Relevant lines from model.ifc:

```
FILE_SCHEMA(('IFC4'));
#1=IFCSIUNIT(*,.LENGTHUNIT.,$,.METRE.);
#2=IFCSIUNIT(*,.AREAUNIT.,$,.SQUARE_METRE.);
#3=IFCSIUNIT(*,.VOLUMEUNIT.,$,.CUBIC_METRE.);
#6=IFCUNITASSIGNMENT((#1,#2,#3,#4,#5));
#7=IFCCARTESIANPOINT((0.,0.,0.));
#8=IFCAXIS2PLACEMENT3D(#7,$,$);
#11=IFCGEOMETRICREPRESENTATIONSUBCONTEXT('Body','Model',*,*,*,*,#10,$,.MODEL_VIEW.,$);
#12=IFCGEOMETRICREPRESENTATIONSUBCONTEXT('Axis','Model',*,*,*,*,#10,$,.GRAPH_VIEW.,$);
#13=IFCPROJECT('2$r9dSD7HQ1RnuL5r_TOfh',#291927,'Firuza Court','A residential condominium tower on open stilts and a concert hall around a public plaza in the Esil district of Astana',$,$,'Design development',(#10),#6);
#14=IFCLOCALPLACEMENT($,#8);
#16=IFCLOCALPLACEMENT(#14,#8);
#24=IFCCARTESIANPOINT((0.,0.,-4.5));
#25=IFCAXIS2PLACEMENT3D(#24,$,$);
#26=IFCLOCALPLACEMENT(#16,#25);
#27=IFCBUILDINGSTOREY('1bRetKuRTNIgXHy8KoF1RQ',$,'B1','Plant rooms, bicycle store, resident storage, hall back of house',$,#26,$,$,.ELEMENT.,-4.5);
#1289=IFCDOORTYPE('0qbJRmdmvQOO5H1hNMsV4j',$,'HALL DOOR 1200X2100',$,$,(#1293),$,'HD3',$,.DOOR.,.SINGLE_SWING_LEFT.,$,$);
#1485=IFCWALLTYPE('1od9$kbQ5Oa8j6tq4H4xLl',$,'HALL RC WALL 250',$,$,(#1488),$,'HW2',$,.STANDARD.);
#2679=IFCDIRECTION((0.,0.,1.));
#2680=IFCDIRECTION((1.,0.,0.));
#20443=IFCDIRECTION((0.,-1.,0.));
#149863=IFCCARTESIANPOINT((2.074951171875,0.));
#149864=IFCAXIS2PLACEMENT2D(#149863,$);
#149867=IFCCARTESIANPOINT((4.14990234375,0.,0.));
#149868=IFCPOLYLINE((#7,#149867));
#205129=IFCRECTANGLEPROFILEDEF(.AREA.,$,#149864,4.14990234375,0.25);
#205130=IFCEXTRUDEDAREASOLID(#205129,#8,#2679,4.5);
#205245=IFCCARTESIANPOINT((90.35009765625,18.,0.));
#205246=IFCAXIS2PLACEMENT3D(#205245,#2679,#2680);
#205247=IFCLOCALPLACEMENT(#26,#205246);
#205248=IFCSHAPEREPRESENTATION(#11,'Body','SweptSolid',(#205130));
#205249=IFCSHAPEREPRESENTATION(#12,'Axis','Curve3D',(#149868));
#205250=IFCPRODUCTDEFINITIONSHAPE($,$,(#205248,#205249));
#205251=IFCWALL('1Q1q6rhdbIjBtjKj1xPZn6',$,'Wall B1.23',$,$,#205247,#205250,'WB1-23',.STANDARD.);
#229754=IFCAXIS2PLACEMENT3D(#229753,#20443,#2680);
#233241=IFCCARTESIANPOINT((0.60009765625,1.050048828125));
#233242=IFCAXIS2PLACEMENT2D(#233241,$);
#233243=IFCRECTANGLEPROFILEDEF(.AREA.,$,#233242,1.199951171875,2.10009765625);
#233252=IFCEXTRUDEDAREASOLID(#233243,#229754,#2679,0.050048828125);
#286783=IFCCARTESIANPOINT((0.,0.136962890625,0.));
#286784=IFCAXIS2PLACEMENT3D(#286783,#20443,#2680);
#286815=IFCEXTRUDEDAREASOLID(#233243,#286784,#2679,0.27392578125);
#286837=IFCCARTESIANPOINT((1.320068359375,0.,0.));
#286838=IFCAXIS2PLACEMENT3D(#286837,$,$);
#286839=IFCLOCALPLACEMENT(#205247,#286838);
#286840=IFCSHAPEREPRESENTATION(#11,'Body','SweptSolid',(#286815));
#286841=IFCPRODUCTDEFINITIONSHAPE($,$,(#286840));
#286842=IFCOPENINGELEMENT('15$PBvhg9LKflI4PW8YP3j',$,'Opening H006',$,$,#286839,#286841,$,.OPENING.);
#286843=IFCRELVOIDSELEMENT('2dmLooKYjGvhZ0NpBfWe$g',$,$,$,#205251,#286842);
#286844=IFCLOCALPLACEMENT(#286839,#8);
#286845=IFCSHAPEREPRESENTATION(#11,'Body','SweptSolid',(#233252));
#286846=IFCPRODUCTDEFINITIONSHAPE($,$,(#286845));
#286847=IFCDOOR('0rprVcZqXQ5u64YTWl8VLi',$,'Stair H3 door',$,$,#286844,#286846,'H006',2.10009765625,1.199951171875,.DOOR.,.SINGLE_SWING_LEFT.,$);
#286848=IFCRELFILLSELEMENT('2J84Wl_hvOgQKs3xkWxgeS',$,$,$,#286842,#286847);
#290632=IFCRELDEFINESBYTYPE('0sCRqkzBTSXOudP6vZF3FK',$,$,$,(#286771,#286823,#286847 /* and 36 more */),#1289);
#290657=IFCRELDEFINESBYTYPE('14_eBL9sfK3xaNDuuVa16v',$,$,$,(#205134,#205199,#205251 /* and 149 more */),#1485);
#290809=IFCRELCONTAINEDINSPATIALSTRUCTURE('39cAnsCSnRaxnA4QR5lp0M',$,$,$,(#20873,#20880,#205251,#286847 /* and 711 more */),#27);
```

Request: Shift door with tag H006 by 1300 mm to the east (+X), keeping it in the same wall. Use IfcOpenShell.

```python
import ifcopenshell
import ifcopenshell.api.geometry
import ifcopenshell.util.placement
import ifcopenshell.util.unit

model = ifcopenshell.open("model.ifc")
unit_scale = ifcopenshell.util.unit.calculate_unit_scale(model)

door = model.by_guid("0rprVcZqXQ5u64YTWl8VLi")
opening = door.FillsVoids[0].RelatingOpeningElement
wall = opening.VoidsElements[0].RelatingBuildingElement

wall_matrix = ifcopenshell.util.placement.get_local_placement(wall.ObjectPlacement)
shift = wall_matrix[:3, 0] * 1.3 / unit_scale
before = ifcopenshell.util.placement.get_local_placement(door.ObjectPlacement)[:3, 3].copy()

# The door is placed relative to its opening, so it follows when the opening moves.
matrix = ifcopenshell.util.placement.get_local_placement(opening.ObjectPlacement)
matrix[:3, 3] += shift
ifcopenshell.api.geometry.edit_object_placement(
    model, product=opening, matrix=matrix, is_si=False, should_transform_children=True
)

after = ifcopenshell.util.placement.get_local_placement(door.ObjectPlacement)[:3, 3]
print("door moved by", (after - before).round(3) + 0.0)

model.write("model_edited.ifc")
```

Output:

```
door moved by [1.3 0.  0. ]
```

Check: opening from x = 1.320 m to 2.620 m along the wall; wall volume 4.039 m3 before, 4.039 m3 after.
